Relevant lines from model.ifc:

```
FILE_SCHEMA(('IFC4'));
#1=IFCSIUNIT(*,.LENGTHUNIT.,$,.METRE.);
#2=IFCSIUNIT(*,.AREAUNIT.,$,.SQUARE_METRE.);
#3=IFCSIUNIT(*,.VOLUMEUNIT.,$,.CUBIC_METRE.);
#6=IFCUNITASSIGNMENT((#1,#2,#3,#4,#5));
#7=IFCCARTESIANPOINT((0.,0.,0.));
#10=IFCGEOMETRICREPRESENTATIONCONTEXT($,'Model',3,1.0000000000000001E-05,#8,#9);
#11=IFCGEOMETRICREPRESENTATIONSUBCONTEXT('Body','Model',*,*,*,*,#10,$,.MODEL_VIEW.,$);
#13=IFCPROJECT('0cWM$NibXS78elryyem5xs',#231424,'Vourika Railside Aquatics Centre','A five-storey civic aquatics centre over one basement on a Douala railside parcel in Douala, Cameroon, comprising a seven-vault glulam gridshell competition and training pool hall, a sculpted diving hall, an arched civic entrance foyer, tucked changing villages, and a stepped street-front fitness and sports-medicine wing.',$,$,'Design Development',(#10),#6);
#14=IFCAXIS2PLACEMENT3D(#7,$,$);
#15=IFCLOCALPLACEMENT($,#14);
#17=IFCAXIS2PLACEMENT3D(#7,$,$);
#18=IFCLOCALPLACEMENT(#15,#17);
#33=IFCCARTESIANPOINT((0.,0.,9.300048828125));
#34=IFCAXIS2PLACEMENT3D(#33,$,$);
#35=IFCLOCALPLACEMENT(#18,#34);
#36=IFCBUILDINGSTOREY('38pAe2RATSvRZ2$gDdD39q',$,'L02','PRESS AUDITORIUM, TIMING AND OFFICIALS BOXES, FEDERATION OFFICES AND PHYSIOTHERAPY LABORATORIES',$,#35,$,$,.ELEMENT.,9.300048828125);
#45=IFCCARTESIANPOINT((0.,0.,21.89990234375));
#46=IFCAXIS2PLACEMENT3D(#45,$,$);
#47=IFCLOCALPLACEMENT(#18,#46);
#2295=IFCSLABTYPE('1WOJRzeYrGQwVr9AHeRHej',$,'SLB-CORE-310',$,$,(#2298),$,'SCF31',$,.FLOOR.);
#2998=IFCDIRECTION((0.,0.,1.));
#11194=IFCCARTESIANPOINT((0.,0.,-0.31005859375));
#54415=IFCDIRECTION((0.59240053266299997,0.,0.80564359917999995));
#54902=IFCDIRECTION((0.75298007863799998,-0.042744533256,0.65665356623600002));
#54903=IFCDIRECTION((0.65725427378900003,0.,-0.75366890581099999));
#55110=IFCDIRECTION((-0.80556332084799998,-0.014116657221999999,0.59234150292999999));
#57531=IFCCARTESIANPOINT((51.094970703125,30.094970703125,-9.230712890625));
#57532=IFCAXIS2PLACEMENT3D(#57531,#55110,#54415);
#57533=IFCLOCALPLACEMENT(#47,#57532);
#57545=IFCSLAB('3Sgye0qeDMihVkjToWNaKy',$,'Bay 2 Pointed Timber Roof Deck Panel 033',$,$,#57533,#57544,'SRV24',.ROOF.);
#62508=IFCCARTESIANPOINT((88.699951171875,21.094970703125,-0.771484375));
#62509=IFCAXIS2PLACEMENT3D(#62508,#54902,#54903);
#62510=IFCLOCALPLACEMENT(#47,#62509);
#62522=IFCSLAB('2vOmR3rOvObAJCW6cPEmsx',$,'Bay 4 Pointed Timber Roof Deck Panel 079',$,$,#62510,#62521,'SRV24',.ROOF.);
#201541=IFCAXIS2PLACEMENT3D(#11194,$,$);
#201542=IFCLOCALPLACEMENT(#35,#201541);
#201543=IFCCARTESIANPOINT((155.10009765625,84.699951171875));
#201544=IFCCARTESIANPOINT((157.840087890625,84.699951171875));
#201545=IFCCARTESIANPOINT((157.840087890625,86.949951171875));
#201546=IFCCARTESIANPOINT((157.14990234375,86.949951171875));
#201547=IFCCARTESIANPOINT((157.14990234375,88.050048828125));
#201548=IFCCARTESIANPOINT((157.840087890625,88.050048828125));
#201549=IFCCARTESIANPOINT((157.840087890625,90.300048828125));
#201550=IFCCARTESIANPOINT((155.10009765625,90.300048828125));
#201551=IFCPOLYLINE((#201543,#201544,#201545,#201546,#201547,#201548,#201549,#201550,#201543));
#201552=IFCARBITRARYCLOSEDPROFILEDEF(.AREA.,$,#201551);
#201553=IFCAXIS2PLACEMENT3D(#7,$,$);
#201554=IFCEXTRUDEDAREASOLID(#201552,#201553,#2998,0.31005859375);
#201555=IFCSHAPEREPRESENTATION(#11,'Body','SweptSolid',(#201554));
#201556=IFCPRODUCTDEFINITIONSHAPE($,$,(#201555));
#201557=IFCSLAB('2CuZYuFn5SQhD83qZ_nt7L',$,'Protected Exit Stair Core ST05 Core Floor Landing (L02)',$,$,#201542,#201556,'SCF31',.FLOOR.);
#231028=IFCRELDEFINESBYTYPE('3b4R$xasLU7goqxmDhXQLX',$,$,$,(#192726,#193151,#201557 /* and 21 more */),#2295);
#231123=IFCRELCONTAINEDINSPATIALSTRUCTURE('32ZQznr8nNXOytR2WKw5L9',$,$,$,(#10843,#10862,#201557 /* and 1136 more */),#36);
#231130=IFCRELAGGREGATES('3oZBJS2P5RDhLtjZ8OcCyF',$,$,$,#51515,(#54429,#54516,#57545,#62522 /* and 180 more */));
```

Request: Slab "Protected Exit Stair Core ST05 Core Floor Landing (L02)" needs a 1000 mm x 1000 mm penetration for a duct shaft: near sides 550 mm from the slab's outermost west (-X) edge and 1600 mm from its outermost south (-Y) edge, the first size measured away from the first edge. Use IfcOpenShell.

```python
import numpy as np
import ifcopenshell
import ifcopenshell.api.feature
import ifcopenshell.api.geometry
import ifcopenshell.api.root
import ifcopenshell.geom
import ifcopenshell.util.placement
import ifcopenshell.util.representation
import ifcopenshell.util.shape
import ifcopenshell.util.unit

model = ifcopenshell.open("model.ifc")
unit_scale = ifcopenshell.util.unit.calculate_unit_scale(model)
settings = ifcopenshell.geom.settings()


def volume(element):
    """Net volume in cubic metres, openings subtracted."""
    shape = ifcopenshell.geom.create_shape(settings, element)
    return ifcopenshell.util.shape.get_volume(shape.geometry)


slab = model.by_guid("2CuZYuFn5SQhD83qZ_nt7L")
before = volume(slab)

# Extent in the slab's own axes, in metres. The edges named are its -X and -Y sides.
slab_shape = ifcopenshell.geom.create_shape(settings, slab)
vertices = ifcopenshell.util.shape.get_vertices(slab_shape.geometry)
x_min, y_min, bottom = vertices.min(axis=0)
top = vertices[:, 2].max()

opening = ifcopenshell.api.root.create_entity(model, ifc_class="IfcOpeningElement", name="Duct shaft opening", predefined_type="OPENING")
context = ifcopenshell.util.representation.get_context(model, "Model", "Body", "MODEL_VIEW")
width, depth = 1, 1
outline = [(0.0, 0.0), (width, 0.0), (width, depth), (0.0, depth), (0.0, 0.0)]
# Overshoot both faces by 50 mm so the cut is clean.
shape = ifcopenshell.api.geometry.add_slab_representation(
    model, context=context, depth=top - bottom + 0.1, polyline=outline
)
ifcopenshell.api.geometry.assign_representation(model, product=opening, representation=shape)

matrix = ifcopenshell.util.placement.get_local_placement(slab.ObjectPlacement)
matrix[:, 3] = matrix @ np.append(np.array([x_min + 0.55, y_min + 1.6, bottom - 0.05]) / unit_scale, 1.0)
ifcopenshell.api.geometry.edit_object_placement(model, product=opening, matrix=matrix, is_si=False)
ifcopenshell.api.feature.add_feature(model, feature=opening, element=slab)

after = volume(slab)

print(f"slab volume {before:.3f} -> {after:.3f} m3")

model.write("model_v2.ifc")
```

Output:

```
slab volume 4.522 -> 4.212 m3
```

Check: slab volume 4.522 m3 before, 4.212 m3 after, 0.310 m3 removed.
